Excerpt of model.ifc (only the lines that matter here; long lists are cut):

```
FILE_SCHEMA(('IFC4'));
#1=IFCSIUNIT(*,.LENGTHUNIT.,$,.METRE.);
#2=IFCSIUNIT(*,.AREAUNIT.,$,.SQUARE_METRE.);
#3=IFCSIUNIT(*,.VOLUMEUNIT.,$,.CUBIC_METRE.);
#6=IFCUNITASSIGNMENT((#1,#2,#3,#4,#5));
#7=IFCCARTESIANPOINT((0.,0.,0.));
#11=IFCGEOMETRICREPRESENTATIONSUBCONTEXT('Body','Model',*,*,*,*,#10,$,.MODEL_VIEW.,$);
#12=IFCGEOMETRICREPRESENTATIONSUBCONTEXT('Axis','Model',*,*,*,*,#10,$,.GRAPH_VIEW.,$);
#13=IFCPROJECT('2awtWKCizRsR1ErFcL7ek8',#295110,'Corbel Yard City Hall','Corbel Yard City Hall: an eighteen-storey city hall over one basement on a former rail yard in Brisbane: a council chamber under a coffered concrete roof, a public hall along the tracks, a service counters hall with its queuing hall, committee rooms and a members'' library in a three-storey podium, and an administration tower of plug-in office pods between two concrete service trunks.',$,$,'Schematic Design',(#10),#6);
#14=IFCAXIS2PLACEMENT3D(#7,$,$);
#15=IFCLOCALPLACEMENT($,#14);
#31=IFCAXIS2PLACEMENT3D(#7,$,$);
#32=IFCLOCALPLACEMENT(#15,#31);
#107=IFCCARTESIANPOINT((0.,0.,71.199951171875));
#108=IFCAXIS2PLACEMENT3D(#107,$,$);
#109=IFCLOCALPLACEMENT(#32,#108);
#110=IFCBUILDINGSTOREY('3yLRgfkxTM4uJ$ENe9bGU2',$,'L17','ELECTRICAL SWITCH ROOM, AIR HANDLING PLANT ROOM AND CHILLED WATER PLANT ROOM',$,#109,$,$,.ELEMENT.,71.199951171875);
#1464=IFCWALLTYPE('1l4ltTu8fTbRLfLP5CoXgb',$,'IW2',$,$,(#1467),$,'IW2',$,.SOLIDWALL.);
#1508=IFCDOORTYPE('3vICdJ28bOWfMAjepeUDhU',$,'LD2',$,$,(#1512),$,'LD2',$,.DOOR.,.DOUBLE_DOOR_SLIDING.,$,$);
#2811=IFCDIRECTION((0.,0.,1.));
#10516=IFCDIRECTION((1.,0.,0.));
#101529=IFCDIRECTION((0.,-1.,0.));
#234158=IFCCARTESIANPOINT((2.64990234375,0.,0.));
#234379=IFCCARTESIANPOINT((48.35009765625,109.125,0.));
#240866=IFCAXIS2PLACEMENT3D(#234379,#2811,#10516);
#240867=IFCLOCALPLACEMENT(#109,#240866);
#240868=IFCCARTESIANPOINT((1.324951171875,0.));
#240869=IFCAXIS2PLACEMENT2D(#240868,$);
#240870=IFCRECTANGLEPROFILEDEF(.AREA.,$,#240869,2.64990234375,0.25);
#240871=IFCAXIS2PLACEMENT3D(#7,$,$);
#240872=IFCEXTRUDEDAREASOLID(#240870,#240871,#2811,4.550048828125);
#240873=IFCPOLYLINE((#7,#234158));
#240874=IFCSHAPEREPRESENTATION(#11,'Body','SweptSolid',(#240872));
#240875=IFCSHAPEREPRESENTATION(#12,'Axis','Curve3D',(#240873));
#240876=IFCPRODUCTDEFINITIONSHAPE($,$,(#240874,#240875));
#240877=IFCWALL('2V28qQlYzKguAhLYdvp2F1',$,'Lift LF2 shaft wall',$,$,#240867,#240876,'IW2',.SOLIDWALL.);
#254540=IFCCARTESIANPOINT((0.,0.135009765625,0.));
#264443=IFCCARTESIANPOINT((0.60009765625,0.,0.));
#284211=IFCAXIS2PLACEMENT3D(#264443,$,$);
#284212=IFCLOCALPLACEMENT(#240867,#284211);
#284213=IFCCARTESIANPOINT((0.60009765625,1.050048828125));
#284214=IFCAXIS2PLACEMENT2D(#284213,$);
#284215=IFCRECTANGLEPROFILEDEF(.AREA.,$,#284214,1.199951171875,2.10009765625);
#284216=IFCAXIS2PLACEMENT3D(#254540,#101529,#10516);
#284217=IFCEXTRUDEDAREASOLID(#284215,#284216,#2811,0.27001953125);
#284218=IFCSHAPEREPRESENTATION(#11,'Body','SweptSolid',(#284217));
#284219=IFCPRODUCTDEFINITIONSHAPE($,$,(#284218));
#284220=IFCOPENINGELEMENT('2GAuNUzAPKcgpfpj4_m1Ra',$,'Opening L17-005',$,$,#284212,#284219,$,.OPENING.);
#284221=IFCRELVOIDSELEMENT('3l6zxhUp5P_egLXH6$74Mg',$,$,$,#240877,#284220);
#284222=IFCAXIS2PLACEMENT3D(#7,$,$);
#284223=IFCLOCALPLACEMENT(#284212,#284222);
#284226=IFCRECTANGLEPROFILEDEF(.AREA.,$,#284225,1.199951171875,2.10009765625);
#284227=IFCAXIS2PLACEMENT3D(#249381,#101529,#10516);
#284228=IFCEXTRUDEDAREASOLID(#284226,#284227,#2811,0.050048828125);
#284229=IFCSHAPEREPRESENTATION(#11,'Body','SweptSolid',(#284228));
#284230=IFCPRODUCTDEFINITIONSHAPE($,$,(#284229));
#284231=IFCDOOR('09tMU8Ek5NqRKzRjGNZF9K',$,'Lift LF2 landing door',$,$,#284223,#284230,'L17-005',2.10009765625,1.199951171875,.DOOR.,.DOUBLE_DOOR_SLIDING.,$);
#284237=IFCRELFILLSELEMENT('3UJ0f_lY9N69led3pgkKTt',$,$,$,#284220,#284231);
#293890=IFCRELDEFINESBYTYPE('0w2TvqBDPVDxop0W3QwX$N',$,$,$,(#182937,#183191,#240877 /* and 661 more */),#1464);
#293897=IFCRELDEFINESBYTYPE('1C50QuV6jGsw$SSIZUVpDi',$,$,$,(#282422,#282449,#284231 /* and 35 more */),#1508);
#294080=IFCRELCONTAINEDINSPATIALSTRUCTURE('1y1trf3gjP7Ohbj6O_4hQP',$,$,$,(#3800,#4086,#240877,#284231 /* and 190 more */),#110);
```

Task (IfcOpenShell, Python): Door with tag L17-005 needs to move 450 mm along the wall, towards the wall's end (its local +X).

```python
import ifcopenshell
import ifcopenshell.api.geometry
import ifcopenshell.util.placement
import ifcopenshell.util.unit

model = ifcopenshell.open("model.ifc")
unit_scale = ifcopenshell.util.unit.calculate_unit_scale(model)

door = model.by_guid("09tMU8Ek5NqRKzRjGNZF9K")
opening = door.FillsVoids[0].RelatingOpeningElement
wall = opening.VoidsElements[0].RelatingBuildingElement

wall_matrix = ifcopenshell.util.placement.get_local_placement(wall.ObjectPlacement)
shift = wall_matrix[:3, 0] * 0.45 / unit_scale
before = ifcopenshell.util.placement.get_local_placement(door.ObjectPlacement)[:3, 3].copy()

# The door is placed relative to its opening, so it follows when the opening moves.
matrix = ifcopenshell.util.placement.get_local_placement(opening.ObjectPlacement)
matrix[:3, 3] += shift
ifcopenshell.api.geometry.edit_object_placement(
    model, product=opening, matrix=matrix, is_si=False, should_transform_children=True
)

after = ifcopenshell.util.placement.get_local_placement(door.ObjectPlacement)[:3, 3]
print("door moved by", (after - before).round(3) + 0.0)

model.write("model-out.ifc")
```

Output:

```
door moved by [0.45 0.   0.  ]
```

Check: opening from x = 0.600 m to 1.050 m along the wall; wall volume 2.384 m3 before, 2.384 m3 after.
